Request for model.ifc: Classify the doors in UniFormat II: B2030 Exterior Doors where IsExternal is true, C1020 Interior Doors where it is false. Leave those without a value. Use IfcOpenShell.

First a look at what the model holds.

```python
import ifcopenshell
import ifcopenshell.util.element

model = ifcopenshell.open("model.ifc")
print(model.schema)
print("classifications:", [c.Name for c in model.by_type("IfcClassification")])
values = [ifcopenshell.util.element.get_pset(e, "Pset_DoorCommon", "IsExternal") for e in model.by_type("IfcDoor")]
for value in (True, False, None):
    print("IsExternal", value, values.count(value))
```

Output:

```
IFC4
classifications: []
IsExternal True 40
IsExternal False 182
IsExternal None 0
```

```python
import ifcopenshell
import ifcopenshell.api.classification
import ifcopenshell.util.element

model = ifcopenshell.open("model.ifc")

system = ifcopenshell.api.classification.add_classification(model, classification="UniFormat II")

doors = model.by_type("IfcDoor")
external = {e: ifcopenshell.util.element.get_pset(e, "Pset_DoorCommon", "IsExternal") for e in doors}
for flag, code, name in ((True, "B2030", "Exterior Doors"), (False, "C1020", "Interior Doors")):
    products = [e for e in doors if external[e] is flag]
    ifcopenshell.api.classification.add_reference(
        model, products=products, classification=system, identification=code, name=name
    )
    print(code, len(products))

model.write("model_v2.ifc")
```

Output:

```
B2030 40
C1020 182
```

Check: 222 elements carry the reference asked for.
